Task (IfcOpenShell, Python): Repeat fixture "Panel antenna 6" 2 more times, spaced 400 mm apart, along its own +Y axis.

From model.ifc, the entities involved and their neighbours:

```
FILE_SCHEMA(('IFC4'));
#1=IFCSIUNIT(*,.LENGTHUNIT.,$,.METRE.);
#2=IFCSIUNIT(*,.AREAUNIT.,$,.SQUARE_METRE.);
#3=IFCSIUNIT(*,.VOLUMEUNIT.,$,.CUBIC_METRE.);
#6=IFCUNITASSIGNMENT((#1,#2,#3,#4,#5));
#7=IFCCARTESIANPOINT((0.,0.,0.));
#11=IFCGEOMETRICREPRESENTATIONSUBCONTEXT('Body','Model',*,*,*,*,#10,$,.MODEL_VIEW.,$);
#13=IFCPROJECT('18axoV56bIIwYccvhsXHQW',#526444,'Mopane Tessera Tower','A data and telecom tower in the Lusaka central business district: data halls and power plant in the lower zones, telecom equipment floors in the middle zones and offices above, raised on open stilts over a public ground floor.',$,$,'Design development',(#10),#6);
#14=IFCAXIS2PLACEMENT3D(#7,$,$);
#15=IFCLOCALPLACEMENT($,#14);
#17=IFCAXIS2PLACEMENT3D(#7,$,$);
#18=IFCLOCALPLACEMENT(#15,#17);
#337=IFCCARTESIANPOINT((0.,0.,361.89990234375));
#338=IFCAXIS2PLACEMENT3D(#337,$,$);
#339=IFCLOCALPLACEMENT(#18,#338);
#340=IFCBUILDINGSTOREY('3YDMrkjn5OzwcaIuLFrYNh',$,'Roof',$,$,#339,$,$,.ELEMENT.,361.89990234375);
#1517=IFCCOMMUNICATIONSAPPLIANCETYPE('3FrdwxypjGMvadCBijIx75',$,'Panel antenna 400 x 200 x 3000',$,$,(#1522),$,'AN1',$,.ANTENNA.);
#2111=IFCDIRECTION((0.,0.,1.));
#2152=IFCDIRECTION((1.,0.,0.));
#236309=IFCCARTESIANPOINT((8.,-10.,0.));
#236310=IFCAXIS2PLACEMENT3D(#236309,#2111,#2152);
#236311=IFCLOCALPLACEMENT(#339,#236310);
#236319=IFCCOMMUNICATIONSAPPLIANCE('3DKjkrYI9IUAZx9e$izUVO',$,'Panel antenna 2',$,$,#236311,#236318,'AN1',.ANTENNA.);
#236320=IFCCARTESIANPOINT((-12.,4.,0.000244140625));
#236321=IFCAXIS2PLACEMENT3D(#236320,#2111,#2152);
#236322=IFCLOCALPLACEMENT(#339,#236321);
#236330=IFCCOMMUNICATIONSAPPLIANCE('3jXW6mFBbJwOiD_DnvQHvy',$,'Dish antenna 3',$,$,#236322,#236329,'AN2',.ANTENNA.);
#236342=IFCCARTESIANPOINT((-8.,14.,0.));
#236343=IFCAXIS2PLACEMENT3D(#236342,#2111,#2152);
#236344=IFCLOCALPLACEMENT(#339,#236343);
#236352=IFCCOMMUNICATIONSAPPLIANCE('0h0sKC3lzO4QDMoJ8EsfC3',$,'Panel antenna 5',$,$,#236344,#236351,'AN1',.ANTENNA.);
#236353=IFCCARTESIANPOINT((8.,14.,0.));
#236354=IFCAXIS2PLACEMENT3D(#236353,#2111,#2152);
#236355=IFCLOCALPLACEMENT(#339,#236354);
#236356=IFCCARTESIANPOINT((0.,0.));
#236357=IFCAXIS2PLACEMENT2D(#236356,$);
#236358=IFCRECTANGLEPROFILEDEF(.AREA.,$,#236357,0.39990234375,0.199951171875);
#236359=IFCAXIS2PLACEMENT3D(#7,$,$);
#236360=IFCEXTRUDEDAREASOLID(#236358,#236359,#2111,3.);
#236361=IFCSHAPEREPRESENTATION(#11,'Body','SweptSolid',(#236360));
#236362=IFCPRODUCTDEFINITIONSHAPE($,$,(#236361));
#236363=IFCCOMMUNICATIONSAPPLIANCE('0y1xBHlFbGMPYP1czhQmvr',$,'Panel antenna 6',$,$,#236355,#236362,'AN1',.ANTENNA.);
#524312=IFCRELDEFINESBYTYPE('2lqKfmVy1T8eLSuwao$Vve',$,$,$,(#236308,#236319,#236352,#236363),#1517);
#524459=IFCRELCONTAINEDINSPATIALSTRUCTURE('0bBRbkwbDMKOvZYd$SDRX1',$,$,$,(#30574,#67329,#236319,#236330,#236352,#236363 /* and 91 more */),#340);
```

```python
import ifcopenshell
import ifcopenshell.api.geometry
import ifcopenshell.api.root
import ifcopenshell.util.element
import ifcopenshell.util.placement
import ifcopenshell.util.unit

model = ifcopenshell.open("model.ifc")
unit_scale = ifcopenshell.util.unit.calculate_unit_scale(model)

source = model.by_guid("0y1xBHlFbGMPYP1czhQmvr")
base = ifcopenshell.util.placement.get_local_placement(source.ObjectPlacement)
step = base[:3, 1] * 0.4 / unit_scale

for i in range(1, 3):
    copy = ifcopenshell.api.root.copy_class(model, product=source)
    copy.Representation = ifcopenshell.util.element.copy_deep(
        model, source.Representation, exclude=["IfcGeometricRepresentationContext", "IfcRepresentationMap"]
    )
    copy.Tag = None
    matrix = base.copy()
    matrix[:3, 3] += i * step
    print("added at", matrix[:3, 3].round(3) + 0.0)
    ifcopenshell.api.geometry.edit_object_placement(model, product=copy, matrix=matrix, is_si=False)

model.write("model_rev.ifc")
```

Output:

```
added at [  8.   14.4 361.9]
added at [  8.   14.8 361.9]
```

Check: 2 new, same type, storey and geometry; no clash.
